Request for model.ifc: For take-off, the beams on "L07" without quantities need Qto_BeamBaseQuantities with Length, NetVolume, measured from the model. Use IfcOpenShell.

First a look at what the model holds.

```python
import ifcopenshell
import ifcopenshell.util.element
import ifcopenshell.util.unit

model = ifcopenshell.open("model.ifc")
print(model.schema)
for unit_type in ("LENGTHUNIT", "AREAUNIT", "VOLUMEUNIT"):
    print(unit_type, ifcopenshell.util.unit.calculate_unit_scale(model, unit_type))
storey = next(s for s in model.by_type("IfcBuildingStorey") if s.Name == "L07")
beams = [e for e in ifcopenshell.util.element.get_decomposition(storey) if e.is_a("IfcBeam")]
for e in sorted(beams, key=lambda e: e.id()):
    print(e.id(), e.is_a(), e.Name, list(ifcopenshell.util.element.get_psets(e, qtos_only=True)), sep=" | ")
```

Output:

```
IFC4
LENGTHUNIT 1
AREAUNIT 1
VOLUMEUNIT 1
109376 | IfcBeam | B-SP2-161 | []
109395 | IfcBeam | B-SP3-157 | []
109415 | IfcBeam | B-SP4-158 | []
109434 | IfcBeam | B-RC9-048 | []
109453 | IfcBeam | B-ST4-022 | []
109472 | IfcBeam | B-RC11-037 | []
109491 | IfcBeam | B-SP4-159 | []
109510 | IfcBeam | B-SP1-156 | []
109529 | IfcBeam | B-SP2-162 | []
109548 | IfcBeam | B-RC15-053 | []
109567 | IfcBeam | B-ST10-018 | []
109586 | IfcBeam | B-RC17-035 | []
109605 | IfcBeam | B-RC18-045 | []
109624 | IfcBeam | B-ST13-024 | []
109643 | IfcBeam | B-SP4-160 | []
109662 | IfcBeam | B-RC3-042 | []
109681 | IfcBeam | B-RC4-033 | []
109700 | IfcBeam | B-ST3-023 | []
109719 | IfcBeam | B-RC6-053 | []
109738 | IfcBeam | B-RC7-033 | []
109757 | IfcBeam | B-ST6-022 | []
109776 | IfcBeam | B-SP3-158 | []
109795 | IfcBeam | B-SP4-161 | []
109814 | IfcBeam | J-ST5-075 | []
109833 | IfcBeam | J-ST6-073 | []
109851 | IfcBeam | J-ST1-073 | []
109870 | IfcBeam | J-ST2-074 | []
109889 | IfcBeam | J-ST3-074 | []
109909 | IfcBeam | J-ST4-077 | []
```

```python
import ifcopenshell
import ifcopenshell.api.pset
import ifcopenshell.geom
import ifcopenshell.util.element
import ifcopenshell.util.shape
import ifcopenshell.util.unit

model = ifcopenshell.open("model.ifc")
unit_scale = ifcopenshell.util.unit.calculate_unit_scale(model)
volume_scale = ifcopenshell.util.unit.calculate_unit_scale(model, "VOLUMEUNIT")
settings = ifcopenshell.geom.settings()

storey = next(s for s in model.by_type("IfcBuildingStorey") if s.Name == "L07")
beams = [e for e in ifcopenshell.util.element.get_decomposition(storey) if e.is_a("IfcBeam")]

for e in sorted(beams, key=lambda e: e.id()):
    if ifcopenshell.util.element.get_psets(e, qtos_only=True, should_inherit=False):
        continue
    # Geometry comes back in metres, in the element's own axes.
    shape = ifcopenshell.geom.create_shape(settings, e)
    values = {
        "Length": ifcopenshell.util.shape.get_max_xyz(shape.geometry) / unit_scale,
        "NetVolume": ifcopenshell.util.shape.get_volume(shape.geometry) / volume_scale,
    }
    qto = ifcopenshell.api.pset.add_qto(model, product=e, name="Qto_BeamBaseQuantities")
    ifcopenshell.api.pset.edit_qto(model, qto=qto, properties=values)
    print(e.id(), {k: round(v, 3) for k, v in values.items()})

model.write("model_updated.ifc")
```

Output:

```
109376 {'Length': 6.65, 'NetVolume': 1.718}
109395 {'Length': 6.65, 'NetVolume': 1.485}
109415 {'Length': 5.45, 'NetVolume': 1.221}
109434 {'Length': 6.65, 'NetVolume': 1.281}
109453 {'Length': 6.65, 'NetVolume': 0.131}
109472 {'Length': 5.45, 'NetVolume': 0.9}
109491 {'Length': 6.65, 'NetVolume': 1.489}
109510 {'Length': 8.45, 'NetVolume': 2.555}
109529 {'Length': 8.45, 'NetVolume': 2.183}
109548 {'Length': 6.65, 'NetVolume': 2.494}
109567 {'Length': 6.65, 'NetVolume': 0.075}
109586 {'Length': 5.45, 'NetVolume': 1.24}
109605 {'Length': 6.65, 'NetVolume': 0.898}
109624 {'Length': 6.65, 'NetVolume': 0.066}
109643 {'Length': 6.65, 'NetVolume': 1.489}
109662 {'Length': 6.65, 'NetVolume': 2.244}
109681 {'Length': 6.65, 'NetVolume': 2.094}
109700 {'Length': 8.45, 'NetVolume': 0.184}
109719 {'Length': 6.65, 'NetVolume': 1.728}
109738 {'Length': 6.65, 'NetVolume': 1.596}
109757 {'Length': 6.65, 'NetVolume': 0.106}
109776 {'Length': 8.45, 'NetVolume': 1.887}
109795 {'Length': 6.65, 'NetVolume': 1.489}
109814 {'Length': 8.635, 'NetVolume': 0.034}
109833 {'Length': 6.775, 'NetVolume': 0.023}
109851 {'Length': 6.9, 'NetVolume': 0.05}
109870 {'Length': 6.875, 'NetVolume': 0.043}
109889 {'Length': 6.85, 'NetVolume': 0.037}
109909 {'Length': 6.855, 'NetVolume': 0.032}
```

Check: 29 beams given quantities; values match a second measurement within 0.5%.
